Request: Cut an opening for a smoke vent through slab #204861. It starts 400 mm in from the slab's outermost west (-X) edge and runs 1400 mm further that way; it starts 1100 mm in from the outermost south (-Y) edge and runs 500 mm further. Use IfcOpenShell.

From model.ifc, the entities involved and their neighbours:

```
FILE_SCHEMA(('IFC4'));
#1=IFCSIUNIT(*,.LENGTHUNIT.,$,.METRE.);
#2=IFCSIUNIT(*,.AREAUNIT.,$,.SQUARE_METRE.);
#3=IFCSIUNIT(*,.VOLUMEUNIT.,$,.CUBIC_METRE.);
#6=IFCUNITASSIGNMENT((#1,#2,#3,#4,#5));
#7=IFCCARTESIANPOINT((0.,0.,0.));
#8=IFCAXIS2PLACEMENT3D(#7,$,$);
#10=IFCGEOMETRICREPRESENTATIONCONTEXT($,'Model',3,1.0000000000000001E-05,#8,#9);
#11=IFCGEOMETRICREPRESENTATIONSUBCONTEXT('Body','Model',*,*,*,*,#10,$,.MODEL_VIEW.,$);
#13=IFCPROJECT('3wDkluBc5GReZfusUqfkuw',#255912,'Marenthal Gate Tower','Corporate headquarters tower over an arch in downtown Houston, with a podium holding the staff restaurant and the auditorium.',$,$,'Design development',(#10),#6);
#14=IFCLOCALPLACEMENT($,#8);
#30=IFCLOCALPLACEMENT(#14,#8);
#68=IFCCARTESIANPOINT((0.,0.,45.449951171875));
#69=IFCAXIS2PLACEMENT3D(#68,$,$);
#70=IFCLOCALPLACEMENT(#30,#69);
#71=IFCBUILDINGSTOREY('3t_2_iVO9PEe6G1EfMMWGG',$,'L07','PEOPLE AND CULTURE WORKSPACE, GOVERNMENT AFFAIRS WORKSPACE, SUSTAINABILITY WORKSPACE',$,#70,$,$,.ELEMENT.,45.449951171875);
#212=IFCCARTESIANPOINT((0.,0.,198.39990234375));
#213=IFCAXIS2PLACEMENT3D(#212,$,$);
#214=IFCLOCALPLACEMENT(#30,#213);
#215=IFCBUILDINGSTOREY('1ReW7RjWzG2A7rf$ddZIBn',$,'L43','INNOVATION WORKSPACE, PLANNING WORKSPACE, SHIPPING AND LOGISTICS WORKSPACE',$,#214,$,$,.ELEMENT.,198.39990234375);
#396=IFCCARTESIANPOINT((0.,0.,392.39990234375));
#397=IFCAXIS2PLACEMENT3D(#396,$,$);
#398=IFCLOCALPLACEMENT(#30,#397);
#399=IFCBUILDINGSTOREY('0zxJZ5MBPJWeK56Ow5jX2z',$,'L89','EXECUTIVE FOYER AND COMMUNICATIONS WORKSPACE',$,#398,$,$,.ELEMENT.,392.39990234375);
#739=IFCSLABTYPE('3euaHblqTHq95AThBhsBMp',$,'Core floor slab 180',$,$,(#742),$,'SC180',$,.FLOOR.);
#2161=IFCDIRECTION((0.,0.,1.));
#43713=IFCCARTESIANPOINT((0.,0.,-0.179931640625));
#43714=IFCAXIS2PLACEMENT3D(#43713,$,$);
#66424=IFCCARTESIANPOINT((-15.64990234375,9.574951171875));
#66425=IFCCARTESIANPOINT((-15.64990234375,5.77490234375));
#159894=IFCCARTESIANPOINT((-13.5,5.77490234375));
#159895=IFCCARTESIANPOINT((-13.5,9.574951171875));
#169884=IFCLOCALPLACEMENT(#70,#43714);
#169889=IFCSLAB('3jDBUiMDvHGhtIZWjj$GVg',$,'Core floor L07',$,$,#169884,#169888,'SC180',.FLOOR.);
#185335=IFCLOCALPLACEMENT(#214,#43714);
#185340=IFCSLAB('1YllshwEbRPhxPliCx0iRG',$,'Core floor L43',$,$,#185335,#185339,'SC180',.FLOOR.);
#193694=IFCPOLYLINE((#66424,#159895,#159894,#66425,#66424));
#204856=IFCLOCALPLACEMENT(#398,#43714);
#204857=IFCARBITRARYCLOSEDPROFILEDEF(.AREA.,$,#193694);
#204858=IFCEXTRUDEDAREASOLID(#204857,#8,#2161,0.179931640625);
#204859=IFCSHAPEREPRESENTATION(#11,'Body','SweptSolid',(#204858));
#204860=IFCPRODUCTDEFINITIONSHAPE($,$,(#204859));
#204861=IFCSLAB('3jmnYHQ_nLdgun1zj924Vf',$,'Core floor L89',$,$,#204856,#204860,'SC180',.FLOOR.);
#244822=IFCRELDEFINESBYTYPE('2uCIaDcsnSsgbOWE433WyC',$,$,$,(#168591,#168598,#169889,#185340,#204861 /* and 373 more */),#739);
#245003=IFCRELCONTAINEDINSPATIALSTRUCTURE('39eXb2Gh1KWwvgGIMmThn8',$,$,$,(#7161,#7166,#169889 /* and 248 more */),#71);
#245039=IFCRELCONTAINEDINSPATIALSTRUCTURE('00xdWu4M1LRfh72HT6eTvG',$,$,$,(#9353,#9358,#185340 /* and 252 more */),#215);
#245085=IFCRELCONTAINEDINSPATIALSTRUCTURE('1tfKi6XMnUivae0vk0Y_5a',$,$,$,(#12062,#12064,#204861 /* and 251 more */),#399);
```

```python
import numpy as np
import ifcopenshell
import ifcopenshell.api.feature
import ifcopenshell.api.geometry
import ifcopenshell.api.root
import ifcopenshell.geom
import ifcopenshell.util.placement
import ifcopenshell.util.representation
import ifcopenshell.util.shape
import ifcopenshell.util.unit

model = ifcopenshell.open("model.ifc")
unit_scale = ifcopenshell.util.unit.calculate_unit_scale(model)
settings = ifcopenshell.geom.settings()


def volume(element):
    """Net volume in cubic metres, openings subtracted."""
    shape = ifcopenshell.geom.create_shape(settings, element)
    return ifcopenshell.util.shape.get_volume(shape.geometry)


slab = model.by_id(204861)
before = volume(slab)

# Extent in the slab's own axes, in metres. The edges named are its -X and -Y sides.
slab_shape = ifcopenshell.geom.create_shape(settings, slab)
vertices = ifcopenshell.util.shape.get_vertices(slab_shape.geometry)
x_min, y_min, bottom = vertices.min(axis=0)
top = vertices[:, 2].max()

opening = ifcopenshell.api.root.create_entity(model, ifc_class="IfcOpeningElement", name="Smoke vent opening", predefined_type="OPENING")
context = ifcopenshell.util.representation.get_context(model, "Model", "Body", "MODEL_VIEW")
width, depth = 1.4, 0.5
outline = [(0.0, 0.0), (width, 0.0), (width, depth), (0.0, depth), (0.0, 0.0)]
# Overshoot both faces by 50 mm so the cut is clean.
shape = ifcopenshell.api.geometry.add_slab_representation(
    model, context=context, depth=top - bottom + 0.1, polyline=outline
)
ifcopenshell.api.geometry.assign_representation(model, product=opening, representation=shape)

matrix = ifcopenshell.util.placement.get_local_placement(slab.ObjectPlacement)
matrix[:, 3] = matrix @ np.append(np.array([x_min + 0.4, y_min + 1.1, bottom - 0.05]) / unit_scale, 1.0)
ifcopenshell.api.geometry.edit_object_placement(model, product=opening, matrix=matrix, is_si=False)
ifcopenshell.api.feature.add_feature(model, feature=opening, element=slab)

after = volume(slab)

print(f"slab volume {before:.3f} -> {after:.3f} m3")

model.write("model-out.ifc")
```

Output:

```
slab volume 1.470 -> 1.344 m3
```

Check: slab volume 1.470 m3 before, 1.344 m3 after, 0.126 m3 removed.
